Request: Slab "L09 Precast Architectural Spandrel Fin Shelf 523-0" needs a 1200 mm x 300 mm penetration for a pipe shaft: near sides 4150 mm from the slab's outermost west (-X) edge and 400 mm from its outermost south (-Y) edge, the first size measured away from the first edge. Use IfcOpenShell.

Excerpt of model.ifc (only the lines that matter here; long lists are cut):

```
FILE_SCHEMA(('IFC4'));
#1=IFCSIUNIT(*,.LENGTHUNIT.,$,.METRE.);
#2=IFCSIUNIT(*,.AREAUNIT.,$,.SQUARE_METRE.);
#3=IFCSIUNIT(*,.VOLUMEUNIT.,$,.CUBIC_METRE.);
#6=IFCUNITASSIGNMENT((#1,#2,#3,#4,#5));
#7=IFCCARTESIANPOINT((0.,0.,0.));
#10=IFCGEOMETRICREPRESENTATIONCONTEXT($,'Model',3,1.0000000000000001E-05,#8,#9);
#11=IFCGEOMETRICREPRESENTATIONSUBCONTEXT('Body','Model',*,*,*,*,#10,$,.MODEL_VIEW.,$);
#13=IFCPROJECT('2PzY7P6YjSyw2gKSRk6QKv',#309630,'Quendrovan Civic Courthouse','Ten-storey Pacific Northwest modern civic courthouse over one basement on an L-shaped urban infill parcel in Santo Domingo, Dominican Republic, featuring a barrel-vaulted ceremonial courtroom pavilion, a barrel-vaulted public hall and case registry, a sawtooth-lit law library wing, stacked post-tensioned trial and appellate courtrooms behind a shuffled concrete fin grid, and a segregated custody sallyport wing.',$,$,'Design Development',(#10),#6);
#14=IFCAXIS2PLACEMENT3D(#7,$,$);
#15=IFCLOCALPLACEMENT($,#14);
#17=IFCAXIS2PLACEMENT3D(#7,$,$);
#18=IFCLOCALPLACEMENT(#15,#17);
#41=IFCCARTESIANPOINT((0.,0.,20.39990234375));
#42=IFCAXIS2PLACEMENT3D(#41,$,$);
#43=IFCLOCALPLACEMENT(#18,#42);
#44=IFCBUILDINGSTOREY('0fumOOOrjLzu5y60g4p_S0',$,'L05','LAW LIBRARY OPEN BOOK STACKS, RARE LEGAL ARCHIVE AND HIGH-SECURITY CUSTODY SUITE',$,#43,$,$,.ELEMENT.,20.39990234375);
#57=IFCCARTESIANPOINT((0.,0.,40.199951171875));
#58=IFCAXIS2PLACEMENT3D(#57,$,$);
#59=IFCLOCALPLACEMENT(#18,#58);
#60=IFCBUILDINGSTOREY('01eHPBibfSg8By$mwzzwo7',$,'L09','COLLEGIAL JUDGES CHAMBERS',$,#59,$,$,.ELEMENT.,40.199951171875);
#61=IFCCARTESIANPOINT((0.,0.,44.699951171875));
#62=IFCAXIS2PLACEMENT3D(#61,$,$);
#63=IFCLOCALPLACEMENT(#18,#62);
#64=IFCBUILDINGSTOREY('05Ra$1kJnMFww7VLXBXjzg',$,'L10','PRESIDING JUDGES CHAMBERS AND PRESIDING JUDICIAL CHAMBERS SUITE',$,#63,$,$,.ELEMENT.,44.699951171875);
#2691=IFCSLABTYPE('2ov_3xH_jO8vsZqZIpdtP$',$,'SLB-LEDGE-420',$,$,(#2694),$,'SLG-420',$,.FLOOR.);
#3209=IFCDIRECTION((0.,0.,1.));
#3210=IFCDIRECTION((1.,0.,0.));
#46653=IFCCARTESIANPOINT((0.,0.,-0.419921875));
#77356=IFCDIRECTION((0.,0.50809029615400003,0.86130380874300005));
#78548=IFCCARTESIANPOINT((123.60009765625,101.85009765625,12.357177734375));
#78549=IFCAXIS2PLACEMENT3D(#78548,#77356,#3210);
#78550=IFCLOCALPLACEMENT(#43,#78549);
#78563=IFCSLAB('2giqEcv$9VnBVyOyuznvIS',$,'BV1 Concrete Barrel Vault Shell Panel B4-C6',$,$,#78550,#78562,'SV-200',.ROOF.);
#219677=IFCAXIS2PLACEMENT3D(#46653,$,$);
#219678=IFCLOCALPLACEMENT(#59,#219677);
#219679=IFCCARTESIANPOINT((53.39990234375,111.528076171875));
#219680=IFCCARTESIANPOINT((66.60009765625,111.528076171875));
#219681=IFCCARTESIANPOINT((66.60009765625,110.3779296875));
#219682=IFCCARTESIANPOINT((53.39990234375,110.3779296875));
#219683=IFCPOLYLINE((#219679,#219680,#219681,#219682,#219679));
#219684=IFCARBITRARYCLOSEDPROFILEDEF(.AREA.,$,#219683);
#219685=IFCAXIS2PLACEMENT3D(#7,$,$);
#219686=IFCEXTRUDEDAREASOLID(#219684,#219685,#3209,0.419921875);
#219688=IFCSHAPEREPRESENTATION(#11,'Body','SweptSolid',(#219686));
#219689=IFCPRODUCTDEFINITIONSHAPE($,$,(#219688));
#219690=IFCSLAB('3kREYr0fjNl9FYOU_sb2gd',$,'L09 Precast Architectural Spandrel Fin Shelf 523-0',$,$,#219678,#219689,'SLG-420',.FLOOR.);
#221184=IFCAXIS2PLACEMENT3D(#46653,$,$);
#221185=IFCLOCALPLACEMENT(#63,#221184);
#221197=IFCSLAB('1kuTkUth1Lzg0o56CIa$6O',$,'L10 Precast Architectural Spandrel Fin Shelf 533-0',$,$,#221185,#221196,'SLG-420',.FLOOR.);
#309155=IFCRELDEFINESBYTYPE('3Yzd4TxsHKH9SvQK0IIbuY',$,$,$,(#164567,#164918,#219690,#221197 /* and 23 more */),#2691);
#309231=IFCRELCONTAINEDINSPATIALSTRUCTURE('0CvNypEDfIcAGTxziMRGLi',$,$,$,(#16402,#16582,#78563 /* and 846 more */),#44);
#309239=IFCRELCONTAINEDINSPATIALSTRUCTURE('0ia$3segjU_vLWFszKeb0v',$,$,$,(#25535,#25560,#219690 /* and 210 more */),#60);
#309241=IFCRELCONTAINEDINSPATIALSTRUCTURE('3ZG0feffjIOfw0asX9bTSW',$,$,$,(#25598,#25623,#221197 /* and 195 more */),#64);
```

```python
import numpy as np
import ifcopenshell
import ifcopenshell.api.feature
import ifcopenshell.api.geometry
import ifcopenshell.api.root
import ifcopenshell.geom
import ifcopenshell.util.placement
import ifcopenshell.util.representation
import ifcopenshell.util.shape
import ifcopenshell.util.unit

model = ifcopenshell.open("model.ifc")
unit_scale = ifcopenshell.util.unit.calculate_unit_scale(model)
settings = ifcopenshell.geom.settings()


def volume(element):
    """Net volume in cubic metres, openings subtracted."""
    shape = ifcopenshell.geom.create_shape(settings, element)
    return ifcopenshell.util.shape.get_volume(shape.geometry)


slab = model.by_guid("3kREYr0fjNl9FYOU_sb2gd")
before = volume(slab)

# Extent in the slab's own axes, in metres. The edges named are its -X and -Y sides.
slab_shape = ifcopenshell.geom.create_shape(settings, slab)
vertices = ifcopenshell.util.shape.get_vertices(slab_shape.geometry)
x_min, y_min, bottom = vertices.min(axis=0)
top = vertices[:, 2].max()

opening = ifcopenshell.api.root.create_entity(model, ifc_class="IfcOpeningElement", name="Pipe shaft opening", predefined_type="OPENING")
context = ifcopenshell.util.representation.get_context(model, "Model", "Body", "MODEL_VIEW")
width, depth = 1.2, 0.3
outline = [(0.0, 0.0), (width, 0.0), (width, depth), (0.0, depth), (0.0, 0.0)]
# Overshoot both faces by 50 mm so the cut is clean.
shape = ifcopenshell.api.geometry.add_slab_representation(
    model, context=context, depth=top - bottom + 0.1, polyline=outline
)
ifcopenshell.api.geometry.assign_representation(model, product=opening, representation=shape)

matrix = ifcopenshell.util.placement.get_local_placement(slab.ObjectPlacement)
matrix[:, 3] = matrix @ np.append(np.array([x_min + 4.15, y_min + 0.4, bottom - 0.05]) / unit_scale, 1.0)
ifcopenshell.api.geometry.edit_object_placement(model, product=opening, matrix=matrix, is_si=False)
ifcopenshell.api.feature.add_feature(model, feature=opening, element=slab)

after = volume(slab)

print(f"slab volume {before:.3f} -> {after:.3f} m3")

model.write("model_rev.ifc")
```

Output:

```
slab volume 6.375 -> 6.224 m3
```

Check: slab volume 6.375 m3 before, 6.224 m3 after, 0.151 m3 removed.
